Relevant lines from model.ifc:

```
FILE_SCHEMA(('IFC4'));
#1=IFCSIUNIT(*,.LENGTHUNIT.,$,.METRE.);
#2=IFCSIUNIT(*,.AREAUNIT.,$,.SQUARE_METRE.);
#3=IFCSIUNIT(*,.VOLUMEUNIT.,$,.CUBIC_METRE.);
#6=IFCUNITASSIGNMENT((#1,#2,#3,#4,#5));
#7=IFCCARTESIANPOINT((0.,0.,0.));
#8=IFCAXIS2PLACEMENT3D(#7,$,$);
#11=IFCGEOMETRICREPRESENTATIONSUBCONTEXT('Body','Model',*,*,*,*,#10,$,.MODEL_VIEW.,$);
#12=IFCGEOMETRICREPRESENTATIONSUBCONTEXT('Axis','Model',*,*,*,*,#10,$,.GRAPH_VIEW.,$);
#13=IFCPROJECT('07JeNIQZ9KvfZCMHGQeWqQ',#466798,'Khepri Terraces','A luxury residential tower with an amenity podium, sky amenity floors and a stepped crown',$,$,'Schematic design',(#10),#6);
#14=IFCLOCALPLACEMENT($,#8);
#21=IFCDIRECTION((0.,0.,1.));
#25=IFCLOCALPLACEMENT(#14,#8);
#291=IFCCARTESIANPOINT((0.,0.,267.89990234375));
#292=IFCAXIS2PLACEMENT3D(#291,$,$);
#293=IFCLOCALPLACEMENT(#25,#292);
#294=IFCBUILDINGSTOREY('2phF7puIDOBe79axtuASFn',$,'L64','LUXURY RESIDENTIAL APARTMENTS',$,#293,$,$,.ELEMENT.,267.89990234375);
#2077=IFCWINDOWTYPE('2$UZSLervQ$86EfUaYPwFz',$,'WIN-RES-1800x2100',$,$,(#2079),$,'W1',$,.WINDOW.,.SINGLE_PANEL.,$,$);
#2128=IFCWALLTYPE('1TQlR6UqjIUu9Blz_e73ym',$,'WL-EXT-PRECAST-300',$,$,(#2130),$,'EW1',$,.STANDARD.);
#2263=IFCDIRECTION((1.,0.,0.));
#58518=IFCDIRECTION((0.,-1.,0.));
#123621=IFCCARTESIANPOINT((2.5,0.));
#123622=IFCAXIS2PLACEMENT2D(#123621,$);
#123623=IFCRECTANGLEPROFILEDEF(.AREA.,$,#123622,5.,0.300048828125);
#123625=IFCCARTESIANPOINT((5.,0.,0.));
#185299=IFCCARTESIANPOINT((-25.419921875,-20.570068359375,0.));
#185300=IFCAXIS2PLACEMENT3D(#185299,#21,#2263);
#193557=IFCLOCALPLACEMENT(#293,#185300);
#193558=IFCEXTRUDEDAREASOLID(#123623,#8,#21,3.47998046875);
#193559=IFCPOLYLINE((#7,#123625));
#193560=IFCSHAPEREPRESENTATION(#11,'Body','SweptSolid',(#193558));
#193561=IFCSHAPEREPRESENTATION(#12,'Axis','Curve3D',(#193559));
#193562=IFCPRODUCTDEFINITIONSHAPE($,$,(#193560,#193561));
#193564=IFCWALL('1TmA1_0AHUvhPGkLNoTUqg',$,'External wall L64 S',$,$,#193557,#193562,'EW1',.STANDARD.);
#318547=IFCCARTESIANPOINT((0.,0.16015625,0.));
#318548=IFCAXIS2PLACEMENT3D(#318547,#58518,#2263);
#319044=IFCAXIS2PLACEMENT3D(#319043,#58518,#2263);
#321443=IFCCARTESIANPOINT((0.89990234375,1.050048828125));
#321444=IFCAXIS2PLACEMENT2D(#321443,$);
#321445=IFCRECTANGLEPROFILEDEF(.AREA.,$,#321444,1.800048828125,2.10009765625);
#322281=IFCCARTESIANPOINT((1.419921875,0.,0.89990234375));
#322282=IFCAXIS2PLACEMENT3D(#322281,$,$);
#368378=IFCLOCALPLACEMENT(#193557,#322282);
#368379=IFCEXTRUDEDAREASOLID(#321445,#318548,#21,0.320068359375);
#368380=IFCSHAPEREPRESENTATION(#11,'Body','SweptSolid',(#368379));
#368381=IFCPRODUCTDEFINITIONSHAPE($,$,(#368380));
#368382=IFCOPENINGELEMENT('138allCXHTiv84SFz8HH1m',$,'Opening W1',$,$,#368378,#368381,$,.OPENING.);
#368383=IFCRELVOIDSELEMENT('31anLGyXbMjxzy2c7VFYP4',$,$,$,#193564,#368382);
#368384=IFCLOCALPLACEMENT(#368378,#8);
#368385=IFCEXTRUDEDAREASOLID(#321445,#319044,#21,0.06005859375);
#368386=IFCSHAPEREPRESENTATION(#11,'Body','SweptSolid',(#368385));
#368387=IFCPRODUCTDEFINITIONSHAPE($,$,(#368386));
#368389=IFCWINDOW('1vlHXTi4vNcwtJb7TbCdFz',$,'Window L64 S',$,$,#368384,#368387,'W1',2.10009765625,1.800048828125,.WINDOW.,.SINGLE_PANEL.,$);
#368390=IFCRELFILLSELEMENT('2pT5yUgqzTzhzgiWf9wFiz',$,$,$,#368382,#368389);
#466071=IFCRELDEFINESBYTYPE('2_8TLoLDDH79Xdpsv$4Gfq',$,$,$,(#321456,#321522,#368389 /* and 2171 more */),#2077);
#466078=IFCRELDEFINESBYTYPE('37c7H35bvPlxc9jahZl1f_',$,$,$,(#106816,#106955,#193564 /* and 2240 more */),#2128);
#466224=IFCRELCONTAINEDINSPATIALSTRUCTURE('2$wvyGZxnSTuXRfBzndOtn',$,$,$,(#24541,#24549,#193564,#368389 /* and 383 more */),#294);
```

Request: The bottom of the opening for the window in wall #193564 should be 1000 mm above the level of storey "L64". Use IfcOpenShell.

```python
import numpy as np
import ifcopenshell
import ifcopenshell.api.geometry
import ifcopenshell.geom
import ifcopenshell.util.element
import ifcopenshell.util.placement
import ifcopenshell.util.shape
import ifcopenshell.util.unit

model = ifcopenshell.open("model.ifc")
unit_scale = ifcopenshell.util.unit.calculate_unit_scale(model)

window = model.by_guid("1vlHXTi4vNcwtJb7TbCdFz")
opening = window.FillsVoids[0].RelatingOpeningElement
storey = ifcopenshell.util.element.get_container(window, ifc_class="IfcBuildingStorey")
level = ifcopenshell.util.placement.get_local_placement(storey.ObjectPlacement)[2, 3]

# The opening's origin need not be at the sill, so measure its lowest point.
shape = ifcopenshell.geom.create_shape(ifcopenshell.geom.settings(), opening)
bottom = ifcopenshell.util.shape.get_shape_bottom_elevation(shape, shape.geometry) / unit_scale
dz = level + 1 / unit_scale - bottom

shift = np.array([0.0, 0.0, dz])
# The window is placed relative to its opening, so it follows when the opening moves.
matrix = ifcopenshell.util.placement.get_local_placement(opening.ObjectPlacement)
matrix[:3, 3] += shift
ifcopenshell.api.geometry.edit_object_placement(
    model, product=opening, matrix=matrix, is_si=False, should_transform_children=True
)

print(f"moved by {dz * unit_scale:+.3f} m")

model.write("model_updated.ifc")
```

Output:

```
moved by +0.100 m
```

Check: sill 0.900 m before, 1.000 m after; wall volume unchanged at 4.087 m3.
